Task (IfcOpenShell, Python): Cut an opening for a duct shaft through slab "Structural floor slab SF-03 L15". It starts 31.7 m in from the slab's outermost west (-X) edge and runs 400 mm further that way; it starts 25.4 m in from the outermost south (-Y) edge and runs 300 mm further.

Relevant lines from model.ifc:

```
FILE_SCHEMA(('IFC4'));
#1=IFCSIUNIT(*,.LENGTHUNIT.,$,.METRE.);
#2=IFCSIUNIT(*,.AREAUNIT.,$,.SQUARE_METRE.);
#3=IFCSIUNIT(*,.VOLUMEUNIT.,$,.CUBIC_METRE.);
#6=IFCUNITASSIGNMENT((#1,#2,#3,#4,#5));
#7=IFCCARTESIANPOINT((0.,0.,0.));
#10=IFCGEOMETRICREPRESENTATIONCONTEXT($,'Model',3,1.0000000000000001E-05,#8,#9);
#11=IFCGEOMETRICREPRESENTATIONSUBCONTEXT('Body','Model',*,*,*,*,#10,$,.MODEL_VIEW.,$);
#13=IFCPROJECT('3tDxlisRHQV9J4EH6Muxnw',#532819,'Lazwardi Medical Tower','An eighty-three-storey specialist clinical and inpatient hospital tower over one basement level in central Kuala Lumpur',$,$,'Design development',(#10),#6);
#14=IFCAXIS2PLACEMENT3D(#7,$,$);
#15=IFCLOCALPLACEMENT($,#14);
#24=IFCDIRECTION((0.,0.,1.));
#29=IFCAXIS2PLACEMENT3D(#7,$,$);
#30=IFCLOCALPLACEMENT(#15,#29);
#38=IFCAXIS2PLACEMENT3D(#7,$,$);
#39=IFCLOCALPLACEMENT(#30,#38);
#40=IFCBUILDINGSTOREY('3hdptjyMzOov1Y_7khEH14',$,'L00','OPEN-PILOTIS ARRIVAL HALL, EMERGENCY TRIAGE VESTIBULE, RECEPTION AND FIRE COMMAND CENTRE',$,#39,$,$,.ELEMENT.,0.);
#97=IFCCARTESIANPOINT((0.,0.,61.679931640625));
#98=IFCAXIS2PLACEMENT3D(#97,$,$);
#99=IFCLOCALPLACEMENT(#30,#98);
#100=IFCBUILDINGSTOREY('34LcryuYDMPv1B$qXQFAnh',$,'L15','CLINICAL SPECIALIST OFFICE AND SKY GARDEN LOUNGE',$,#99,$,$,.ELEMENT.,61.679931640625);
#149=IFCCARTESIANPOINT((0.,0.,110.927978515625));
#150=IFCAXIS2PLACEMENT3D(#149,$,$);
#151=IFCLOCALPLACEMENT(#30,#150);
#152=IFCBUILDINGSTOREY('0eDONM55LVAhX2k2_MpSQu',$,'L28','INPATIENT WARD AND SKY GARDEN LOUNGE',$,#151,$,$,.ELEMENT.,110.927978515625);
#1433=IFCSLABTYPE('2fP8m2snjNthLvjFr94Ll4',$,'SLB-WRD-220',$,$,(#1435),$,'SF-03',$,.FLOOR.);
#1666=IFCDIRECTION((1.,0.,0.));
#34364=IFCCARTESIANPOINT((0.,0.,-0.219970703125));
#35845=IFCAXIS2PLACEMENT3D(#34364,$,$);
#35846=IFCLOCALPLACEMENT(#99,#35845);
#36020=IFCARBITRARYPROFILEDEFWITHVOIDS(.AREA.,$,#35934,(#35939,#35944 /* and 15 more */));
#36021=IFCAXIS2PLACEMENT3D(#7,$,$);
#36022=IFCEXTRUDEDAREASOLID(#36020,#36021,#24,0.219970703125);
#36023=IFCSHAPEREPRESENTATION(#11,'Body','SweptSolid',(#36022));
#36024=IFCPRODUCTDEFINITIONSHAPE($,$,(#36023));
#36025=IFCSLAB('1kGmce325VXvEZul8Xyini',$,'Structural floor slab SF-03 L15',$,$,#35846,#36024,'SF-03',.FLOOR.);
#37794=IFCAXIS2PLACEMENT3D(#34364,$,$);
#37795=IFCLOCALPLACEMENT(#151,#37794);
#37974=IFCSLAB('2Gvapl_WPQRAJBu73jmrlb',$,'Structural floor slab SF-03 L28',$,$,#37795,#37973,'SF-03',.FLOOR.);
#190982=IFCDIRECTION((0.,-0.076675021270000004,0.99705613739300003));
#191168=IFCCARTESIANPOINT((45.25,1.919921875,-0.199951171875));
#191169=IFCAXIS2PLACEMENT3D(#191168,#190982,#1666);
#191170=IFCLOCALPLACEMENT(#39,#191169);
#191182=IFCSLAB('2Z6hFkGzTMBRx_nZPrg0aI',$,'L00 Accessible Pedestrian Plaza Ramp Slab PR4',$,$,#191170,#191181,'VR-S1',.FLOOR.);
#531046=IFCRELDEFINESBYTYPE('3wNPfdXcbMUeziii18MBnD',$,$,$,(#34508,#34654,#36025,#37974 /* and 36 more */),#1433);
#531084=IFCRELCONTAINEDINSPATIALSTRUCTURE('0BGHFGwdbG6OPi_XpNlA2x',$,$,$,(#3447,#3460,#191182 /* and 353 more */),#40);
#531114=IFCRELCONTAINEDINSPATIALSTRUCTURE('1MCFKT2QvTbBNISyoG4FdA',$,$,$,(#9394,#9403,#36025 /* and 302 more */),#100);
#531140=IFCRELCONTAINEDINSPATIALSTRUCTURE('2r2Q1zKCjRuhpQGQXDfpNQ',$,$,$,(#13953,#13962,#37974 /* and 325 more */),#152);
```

```python
import numpy as np
import ifcopenshell
import ifcopenshell.api.feature
import ifcopenshell.api.geometry
import ifcopenshell.api.root
import ifcopenshell.geom
import ifcopenshell.util.placement
import ifcopenshell.util.representation
import ifcopenshell.util.shape
import ifcopenshell.util.unit

model = ifcopenshell.open("model.ifc")
unit_scale = ifcopenshell.util.unit.calculate_unit_scale(model)
settings = ifcopenshell.geom.settings()


def volume(element):
    """Net volume in cubic metres, openings subtracted."""
    shape = ifcopenshell.geom.create_shape(settings, element)
    return ifcopenshell.util.shape.get_volume(shape.geometry)


slab = model.by_guid("1kGmce325VXvEZul8Xyini")
before = volume(slab)

# Extent in the slab's own axes, in metres. The edges named are its -X and -Y sides.
slab_shape = ifcopenshell.geom.create_shape(settings, slab)
vertices = ifcopenshell.util.shape.get_vertices(slab_shape.geometry)
x_min, y_min, bottom = vertices.min(axis=0)
top = vertices[:, 2].max()

opening = ifcopenshell.api.root.create_entity(model, ifc_class="IfcOpeningElement", name="Duct shaft opening", predefined_type="OPENING")
context = ifcopenshell.util.representation.get_context(model, "Model", "Body", "MODEL_VIEW")
width, depth = 0.4, 0.3
outline = [(0.0, 0.0), (width, 0.0), (width, depth), (0.0, depth), (0.0, 0.0)]
# Overshoot both faces by 50 mm so the cut is clean.
shape = ifcopenshell.api.geometry.add_slab_representation(
    model, context=context, depth=top - bottom + 0.1, polyline=outline
)
ifcopenshell.api.geometry.assign_representation(model, product=opening, representation=shape)

matrix = ifcopenshell.util.placement.get_local_placement(slab.ObjectPlacement)
matrix[:, 3] = matrix @ np.append(np.array([x_min + 31.7, y_min + 25.4, bottom - 0.05]) / unit_scale, 1.0)
ifcopenshell.api.geometry.edit_object_placement(model, product=opening, matrix=matrix, is_si=False)
ifcopenshell.api.feature.add_feature(model, feature=opening, element=slab)

after = volume(slab)

print(f"slab volume {before:.3f} -> {after:.3f} m3")

model.write("model-out.ifc")
```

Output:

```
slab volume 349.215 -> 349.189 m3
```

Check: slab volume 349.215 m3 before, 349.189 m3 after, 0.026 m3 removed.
